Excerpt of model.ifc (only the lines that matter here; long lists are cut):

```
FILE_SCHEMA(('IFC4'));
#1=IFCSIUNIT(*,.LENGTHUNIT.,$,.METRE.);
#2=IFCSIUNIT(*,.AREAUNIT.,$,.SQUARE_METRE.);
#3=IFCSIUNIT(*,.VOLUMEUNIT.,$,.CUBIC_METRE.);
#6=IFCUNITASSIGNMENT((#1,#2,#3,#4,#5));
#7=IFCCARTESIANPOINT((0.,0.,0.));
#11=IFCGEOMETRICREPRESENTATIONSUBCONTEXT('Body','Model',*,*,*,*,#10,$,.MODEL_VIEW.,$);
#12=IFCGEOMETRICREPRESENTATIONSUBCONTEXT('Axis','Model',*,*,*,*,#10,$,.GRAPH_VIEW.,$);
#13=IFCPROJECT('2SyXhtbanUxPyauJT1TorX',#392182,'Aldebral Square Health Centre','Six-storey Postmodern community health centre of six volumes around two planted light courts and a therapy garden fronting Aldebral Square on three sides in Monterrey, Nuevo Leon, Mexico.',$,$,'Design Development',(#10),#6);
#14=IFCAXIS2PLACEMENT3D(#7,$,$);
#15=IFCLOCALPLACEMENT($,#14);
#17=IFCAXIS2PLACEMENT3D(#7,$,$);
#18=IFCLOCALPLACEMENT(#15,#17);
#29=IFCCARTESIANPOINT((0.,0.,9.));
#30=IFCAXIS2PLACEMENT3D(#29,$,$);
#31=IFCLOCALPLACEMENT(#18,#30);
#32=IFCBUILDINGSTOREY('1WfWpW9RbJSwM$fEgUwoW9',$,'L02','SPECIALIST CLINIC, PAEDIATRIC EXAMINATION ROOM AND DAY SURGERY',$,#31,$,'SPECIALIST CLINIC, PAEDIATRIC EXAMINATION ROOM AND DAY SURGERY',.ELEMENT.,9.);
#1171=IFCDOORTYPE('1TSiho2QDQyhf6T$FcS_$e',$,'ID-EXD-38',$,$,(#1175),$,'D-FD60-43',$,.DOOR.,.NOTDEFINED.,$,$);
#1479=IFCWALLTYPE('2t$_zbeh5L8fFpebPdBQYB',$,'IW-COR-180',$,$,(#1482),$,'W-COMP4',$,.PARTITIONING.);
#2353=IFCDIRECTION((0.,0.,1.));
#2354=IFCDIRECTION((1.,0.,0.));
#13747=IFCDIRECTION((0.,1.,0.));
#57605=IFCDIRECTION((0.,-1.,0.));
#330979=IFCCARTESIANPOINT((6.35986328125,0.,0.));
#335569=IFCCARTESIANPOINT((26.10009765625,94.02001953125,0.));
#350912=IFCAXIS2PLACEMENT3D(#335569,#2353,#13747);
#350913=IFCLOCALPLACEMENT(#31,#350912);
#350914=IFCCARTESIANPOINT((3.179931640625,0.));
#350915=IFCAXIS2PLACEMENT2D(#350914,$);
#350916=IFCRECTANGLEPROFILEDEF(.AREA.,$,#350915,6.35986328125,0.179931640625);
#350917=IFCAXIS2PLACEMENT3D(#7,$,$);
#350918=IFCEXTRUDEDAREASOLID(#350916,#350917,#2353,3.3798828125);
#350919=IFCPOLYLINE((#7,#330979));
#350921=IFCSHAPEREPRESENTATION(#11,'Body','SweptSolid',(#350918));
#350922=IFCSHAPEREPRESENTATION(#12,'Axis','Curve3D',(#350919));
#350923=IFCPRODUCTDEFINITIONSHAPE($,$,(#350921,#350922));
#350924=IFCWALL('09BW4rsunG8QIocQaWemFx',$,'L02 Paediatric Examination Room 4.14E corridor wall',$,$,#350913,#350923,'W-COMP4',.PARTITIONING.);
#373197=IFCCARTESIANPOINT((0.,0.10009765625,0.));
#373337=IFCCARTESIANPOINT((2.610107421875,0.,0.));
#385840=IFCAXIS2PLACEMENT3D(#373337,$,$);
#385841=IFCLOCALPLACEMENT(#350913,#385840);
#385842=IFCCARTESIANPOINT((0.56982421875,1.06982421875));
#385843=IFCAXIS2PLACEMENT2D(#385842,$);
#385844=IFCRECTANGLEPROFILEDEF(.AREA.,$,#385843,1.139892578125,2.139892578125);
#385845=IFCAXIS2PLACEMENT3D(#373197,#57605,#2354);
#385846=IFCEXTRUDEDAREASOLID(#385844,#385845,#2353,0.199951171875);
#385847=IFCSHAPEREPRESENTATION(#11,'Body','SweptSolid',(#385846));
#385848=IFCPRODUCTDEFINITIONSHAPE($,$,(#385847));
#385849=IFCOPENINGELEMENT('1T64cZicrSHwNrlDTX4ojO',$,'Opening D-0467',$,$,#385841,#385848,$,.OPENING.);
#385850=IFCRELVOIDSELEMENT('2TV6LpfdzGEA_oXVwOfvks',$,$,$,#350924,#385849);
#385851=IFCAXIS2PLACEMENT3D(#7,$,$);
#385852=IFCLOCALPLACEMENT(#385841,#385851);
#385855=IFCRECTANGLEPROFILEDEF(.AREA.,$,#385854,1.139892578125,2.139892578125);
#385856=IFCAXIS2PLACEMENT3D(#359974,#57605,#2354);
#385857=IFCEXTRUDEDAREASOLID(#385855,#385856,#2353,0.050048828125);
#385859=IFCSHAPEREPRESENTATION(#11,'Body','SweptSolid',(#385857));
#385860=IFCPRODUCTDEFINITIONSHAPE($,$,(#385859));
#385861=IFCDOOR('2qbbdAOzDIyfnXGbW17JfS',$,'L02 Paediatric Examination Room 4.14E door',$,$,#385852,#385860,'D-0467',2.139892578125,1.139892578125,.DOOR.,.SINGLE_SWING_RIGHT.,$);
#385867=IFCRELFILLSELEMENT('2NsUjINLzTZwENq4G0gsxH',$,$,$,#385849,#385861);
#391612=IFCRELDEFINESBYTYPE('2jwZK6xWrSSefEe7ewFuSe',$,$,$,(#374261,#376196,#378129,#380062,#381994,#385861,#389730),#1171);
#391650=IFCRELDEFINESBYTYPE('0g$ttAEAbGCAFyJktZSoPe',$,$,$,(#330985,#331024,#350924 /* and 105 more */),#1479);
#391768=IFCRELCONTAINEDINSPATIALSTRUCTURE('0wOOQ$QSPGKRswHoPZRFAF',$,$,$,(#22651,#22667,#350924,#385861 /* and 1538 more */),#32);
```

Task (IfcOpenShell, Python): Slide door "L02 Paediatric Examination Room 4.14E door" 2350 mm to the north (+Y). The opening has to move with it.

```python
import ifcopenshell
import ifcopenshell.api.geometry
import ifcopenshell.util.placement
import ifcopenshell.util.unit

model = ifcopenshell.open("model.ifc")
unit_scale = ifcopenshell.util.unit.calculate_unit_scale(model)

door = model.by_guid("2qbbdAOzDIyfnXGbW17JfS")
opening = door.FillsVoids[0].RelatingOpeningElement
wall = opening.VoidsElements[0].RelatingBuildingElement

wall_matrix = ifcopenshell.util.placement.get_local_placement(wall.ObjectPlacement)
shift = wall_matrix[:3, 0] * 2.35 / unit_scale
before = ifcopenshell.util.placement.get_local_placement(door.ObjectPlacement)[:3, 3].copy()

# The door is placed relative to its opening, so it follows when the opening moves.
matrix = ifcopenshell.util.placement.get_local_placement(opening.ObjectPlacement)
matrix[:3, 3] += shift
ifcopenshell.api.geometry.edit_object_placement(
    model, product=opening, matrix=matrix, is_si=False, should_transform_children=True
)

after = ifcopenshell.util.placement.get_local_placement(door.ObjectPlacement)[:3, 3]
print("door moved by", (after - before).round(3) + 0.0)

model.write("model_rev.ifc")
```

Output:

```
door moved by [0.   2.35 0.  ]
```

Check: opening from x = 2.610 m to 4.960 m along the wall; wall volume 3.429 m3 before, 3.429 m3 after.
